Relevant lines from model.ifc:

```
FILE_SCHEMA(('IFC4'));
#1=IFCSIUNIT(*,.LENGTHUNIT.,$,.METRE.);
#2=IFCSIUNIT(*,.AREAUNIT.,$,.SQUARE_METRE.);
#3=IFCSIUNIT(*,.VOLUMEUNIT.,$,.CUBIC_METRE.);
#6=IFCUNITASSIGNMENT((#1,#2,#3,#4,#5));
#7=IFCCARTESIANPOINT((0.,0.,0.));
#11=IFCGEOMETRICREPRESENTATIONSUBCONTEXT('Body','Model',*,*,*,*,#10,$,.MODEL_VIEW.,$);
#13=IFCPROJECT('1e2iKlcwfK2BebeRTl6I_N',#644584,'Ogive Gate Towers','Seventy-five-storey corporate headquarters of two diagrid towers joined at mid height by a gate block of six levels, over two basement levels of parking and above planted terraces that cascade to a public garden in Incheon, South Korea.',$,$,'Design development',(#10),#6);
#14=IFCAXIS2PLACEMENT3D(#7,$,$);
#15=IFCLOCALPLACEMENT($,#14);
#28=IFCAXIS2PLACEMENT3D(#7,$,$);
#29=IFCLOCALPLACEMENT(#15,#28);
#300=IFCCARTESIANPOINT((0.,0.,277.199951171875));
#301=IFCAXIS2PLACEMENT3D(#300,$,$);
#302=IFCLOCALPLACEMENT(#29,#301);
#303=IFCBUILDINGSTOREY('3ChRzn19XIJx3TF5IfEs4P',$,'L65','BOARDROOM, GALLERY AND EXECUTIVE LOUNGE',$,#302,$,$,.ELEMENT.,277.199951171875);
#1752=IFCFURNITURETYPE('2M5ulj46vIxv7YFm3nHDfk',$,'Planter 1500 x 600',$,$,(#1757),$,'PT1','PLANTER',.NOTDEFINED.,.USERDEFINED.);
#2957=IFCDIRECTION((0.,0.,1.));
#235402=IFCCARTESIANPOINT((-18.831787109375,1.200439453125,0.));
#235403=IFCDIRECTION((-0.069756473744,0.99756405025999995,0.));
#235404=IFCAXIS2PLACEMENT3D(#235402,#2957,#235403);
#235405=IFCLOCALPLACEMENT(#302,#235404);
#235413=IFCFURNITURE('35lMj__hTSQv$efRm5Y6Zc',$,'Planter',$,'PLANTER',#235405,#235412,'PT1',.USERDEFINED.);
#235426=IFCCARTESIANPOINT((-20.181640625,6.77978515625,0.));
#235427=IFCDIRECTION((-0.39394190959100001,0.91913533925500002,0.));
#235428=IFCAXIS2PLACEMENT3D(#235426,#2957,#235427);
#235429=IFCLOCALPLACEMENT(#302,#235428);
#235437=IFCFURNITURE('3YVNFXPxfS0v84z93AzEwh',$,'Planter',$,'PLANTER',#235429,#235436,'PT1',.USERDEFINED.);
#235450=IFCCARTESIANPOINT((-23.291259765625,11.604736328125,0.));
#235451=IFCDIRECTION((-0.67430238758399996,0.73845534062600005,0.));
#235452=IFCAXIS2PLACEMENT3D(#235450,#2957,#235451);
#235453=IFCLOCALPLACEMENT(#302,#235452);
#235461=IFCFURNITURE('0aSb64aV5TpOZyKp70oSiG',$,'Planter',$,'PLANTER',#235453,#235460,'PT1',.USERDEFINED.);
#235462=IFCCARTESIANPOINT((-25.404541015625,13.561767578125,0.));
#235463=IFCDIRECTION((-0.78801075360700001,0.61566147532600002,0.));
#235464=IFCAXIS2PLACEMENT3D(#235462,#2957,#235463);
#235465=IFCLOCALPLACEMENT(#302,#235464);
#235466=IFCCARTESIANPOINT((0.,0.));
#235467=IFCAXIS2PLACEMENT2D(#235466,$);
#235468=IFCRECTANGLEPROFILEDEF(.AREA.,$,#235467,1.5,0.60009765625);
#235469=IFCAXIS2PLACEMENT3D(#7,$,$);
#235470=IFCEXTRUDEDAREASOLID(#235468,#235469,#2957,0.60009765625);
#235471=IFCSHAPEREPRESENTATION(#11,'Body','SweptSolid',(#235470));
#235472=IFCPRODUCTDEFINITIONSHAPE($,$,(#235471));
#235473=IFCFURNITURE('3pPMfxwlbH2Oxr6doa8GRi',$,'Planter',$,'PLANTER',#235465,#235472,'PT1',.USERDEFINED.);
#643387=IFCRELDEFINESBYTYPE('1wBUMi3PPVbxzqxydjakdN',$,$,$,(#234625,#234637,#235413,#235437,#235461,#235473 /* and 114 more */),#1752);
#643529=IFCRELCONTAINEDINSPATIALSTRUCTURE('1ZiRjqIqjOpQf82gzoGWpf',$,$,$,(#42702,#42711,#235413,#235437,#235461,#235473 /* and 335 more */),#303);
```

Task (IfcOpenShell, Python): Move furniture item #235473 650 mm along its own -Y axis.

```python
import ifcopenshell
import ifcopenshell.api.geometry
import ifcopenshell.util.placement
import ifcopenshell.util.unit

model = ifcopenshell.open("model.ifc")
unit_scale = ifcopenshell.util.unit.calculate_unit_scale(model)

item = model.by_guid("3pPMfxwlbH2Oxr6doa8GRi")
matrix = ifcopenshell.util.placement.get_local_placement(item.ObjectPlacement)
matrix[:3, 3] -= matrix[:3, 1] * 0.65 / unit_scale
ifcopenshell.api.geometry.edit_object_placement(model, product=item, matrix=matrix, is_si=False)

print(ifcopenshell.util.placement.get_local_placement(item.ObjectPlacement).round(3) + 0.0)

model.write("model_updated.ifc")
```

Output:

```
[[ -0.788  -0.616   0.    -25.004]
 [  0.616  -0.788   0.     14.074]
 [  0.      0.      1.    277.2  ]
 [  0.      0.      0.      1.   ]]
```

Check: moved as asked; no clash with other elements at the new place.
